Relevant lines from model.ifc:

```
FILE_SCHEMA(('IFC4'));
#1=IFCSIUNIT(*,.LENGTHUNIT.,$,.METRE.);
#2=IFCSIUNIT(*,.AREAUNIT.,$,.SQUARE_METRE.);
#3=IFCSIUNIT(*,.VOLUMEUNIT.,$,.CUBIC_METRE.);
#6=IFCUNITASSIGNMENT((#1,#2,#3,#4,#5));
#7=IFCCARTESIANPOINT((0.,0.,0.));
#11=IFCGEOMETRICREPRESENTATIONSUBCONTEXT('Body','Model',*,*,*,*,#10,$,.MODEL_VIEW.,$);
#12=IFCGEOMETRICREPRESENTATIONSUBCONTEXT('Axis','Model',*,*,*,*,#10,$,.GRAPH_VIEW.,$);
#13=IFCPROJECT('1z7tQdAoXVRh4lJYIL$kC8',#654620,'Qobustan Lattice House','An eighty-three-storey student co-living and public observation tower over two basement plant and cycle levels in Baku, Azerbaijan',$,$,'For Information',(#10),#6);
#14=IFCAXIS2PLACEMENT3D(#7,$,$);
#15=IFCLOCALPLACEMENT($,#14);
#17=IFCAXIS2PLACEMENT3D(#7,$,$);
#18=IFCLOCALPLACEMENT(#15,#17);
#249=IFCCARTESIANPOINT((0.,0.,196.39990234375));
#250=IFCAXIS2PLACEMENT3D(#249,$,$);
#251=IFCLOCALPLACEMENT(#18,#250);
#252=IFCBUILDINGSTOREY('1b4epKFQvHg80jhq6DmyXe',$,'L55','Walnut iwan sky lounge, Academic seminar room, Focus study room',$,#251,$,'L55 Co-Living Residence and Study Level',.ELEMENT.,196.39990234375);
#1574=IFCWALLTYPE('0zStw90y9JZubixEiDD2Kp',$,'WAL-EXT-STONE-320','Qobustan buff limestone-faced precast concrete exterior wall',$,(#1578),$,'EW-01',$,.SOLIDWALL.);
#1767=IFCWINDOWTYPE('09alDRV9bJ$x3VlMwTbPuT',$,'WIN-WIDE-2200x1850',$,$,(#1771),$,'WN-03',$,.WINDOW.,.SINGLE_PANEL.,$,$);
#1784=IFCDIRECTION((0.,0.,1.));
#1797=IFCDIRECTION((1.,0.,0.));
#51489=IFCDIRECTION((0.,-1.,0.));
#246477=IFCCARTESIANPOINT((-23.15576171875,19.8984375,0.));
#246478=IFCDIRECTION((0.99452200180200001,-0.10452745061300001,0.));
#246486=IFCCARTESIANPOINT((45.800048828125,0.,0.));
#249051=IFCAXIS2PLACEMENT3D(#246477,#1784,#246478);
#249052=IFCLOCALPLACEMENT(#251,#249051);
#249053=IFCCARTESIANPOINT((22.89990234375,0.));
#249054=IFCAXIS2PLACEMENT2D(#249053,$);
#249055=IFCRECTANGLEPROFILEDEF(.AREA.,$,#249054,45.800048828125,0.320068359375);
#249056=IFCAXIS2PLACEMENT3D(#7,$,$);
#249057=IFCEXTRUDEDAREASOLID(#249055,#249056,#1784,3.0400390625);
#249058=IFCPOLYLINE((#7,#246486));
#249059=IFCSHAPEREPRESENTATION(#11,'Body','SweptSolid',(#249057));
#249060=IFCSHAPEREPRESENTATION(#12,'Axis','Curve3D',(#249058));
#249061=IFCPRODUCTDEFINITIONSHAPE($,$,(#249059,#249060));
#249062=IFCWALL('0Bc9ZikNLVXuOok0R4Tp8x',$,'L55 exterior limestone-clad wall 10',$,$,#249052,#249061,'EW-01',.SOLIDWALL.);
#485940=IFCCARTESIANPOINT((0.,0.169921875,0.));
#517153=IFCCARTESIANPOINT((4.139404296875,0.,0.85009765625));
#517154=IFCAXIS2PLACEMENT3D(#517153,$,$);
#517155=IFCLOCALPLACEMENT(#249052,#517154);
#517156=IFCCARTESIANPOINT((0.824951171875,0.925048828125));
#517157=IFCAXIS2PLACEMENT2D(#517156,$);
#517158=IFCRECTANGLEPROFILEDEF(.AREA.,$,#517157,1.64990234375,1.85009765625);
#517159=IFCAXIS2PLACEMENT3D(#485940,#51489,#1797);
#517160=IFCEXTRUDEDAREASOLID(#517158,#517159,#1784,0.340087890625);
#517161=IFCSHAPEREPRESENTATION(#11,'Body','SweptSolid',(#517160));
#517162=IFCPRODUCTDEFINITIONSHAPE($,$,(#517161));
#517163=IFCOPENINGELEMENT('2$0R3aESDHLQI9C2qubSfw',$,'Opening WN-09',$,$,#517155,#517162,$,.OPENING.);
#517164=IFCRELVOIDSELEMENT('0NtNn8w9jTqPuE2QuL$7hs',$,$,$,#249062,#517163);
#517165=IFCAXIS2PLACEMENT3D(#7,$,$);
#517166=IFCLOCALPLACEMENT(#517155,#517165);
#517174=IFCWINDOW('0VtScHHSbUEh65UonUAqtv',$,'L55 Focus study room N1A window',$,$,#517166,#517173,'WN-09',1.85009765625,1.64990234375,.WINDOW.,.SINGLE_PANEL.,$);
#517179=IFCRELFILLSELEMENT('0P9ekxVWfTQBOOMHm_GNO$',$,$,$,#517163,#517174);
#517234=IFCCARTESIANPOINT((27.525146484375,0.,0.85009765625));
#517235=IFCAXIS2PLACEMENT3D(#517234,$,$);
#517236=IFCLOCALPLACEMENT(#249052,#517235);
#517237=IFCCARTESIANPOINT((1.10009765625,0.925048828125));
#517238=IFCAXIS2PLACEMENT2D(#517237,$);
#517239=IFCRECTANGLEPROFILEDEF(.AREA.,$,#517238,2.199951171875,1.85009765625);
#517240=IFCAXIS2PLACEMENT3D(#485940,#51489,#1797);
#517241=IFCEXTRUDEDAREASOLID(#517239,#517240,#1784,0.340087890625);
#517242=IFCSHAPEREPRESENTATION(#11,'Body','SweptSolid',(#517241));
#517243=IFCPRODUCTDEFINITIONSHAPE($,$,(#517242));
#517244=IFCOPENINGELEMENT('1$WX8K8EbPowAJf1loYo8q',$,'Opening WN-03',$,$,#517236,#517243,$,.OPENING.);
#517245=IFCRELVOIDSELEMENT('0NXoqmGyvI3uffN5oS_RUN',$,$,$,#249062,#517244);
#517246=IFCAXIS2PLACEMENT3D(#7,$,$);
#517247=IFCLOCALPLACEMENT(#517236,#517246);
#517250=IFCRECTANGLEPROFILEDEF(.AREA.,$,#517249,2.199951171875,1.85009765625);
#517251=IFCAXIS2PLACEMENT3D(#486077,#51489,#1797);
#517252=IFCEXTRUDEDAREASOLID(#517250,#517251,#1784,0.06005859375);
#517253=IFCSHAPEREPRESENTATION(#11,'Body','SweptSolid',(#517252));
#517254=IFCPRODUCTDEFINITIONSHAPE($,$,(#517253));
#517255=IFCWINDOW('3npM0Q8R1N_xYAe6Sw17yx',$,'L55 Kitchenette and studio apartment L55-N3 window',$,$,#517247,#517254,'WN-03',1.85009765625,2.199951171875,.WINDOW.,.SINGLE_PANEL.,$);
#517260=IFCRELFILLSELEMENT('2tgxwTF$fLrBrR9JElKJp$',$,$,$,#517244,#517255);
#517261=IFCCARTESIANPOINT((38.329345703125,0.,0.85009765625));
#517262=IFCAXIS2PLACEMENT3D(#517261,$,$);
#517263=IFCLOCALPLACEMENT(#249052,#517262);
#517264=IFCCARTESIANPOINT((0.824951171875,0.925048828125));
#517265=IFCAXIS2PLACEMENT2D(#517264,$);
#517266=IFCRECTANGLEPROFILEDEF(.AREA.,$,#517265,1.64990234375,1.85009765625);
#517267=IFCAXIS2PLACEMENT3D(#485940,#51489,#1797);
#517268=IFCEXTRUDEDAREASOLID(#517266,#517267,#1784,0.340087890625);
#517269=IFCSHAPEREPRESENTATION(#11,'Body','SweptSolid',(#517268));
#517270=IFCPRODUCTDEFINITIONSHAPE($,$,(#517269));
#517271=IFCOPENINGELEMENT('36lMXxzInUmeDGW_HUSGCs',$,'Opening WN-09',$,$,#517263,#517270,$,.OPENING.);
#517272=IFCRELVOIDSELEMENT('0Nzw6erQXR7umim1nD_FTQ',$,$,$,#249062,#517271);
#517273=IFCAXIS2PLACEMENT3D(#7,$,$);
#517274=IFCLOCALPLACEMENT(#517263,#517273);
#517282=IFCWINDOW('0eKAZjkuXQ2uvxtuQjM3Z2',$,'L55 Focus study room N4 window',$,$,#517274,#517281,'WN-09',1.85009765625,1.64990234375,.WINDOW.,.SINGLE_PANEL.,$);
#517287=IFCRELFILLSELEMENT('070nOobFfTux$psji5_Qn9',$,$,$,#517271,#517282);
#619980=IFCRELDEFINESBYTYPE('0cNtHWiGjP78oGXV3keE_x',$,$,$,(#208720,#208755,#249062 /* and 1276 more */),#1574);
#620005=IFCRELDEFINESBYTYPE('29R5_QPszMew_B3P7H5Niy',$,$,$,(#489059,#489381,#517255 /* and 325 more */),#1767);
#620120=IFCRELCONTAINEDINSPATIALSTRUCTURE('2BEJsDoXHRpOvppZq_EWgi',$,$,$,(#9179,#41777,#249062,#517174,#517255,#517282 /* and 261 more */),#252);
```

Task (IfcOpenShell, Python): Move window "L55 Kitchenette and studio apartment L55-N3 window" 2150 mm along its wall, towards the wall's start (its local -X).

```python
import ifcopenshell
import ifcopenshell.api.geometry
import ifcopenshell.util.placement
import ifcopenshell.util.unit

model = ifcopenshell.open("model.ifc")
unit_scale = ifcopenshell.util.unit.calculate_unit_scale(model)

window = model.by_id(517255)
opening = window.FillsVoids[0].RelatingOpeningElement
wall = opening.VoidsElements[0].RelatingBuildingElement

wall_matrix = ifcopenshell.util.placement.get_local_placement(wall.ObjectPlacement)
shift = wall_matrix[:3, 0] * -2.15 / unit_scale
before = ifcopenshell.util.placement.get_local_placement(window.ObjectPlacement)[:3, 3].copy()

# The window is placed relative to its opening, so it follows when the opening moves.
matrix = ifcopenshell.util.placement.get_local_placement(opening.ObjectPlacement)
matrix[:3, 3] += shift
ifcopenshell.api.geometry.edit_object_placement(
    model, product=opening, matrix=matrix, is_si=False, should_transform_children=True
)

after = ifcopenshell.util.placement.get_local_placement(window.ObjectPlacement)[:3, 3]
print("window moved by", (after - before).round(3) + 0.0)

model.write("model_updated.ifc")
```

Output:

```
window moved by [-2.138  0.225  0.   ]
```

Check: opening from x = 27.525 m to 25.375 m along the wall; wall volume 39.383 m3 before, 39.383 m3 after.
